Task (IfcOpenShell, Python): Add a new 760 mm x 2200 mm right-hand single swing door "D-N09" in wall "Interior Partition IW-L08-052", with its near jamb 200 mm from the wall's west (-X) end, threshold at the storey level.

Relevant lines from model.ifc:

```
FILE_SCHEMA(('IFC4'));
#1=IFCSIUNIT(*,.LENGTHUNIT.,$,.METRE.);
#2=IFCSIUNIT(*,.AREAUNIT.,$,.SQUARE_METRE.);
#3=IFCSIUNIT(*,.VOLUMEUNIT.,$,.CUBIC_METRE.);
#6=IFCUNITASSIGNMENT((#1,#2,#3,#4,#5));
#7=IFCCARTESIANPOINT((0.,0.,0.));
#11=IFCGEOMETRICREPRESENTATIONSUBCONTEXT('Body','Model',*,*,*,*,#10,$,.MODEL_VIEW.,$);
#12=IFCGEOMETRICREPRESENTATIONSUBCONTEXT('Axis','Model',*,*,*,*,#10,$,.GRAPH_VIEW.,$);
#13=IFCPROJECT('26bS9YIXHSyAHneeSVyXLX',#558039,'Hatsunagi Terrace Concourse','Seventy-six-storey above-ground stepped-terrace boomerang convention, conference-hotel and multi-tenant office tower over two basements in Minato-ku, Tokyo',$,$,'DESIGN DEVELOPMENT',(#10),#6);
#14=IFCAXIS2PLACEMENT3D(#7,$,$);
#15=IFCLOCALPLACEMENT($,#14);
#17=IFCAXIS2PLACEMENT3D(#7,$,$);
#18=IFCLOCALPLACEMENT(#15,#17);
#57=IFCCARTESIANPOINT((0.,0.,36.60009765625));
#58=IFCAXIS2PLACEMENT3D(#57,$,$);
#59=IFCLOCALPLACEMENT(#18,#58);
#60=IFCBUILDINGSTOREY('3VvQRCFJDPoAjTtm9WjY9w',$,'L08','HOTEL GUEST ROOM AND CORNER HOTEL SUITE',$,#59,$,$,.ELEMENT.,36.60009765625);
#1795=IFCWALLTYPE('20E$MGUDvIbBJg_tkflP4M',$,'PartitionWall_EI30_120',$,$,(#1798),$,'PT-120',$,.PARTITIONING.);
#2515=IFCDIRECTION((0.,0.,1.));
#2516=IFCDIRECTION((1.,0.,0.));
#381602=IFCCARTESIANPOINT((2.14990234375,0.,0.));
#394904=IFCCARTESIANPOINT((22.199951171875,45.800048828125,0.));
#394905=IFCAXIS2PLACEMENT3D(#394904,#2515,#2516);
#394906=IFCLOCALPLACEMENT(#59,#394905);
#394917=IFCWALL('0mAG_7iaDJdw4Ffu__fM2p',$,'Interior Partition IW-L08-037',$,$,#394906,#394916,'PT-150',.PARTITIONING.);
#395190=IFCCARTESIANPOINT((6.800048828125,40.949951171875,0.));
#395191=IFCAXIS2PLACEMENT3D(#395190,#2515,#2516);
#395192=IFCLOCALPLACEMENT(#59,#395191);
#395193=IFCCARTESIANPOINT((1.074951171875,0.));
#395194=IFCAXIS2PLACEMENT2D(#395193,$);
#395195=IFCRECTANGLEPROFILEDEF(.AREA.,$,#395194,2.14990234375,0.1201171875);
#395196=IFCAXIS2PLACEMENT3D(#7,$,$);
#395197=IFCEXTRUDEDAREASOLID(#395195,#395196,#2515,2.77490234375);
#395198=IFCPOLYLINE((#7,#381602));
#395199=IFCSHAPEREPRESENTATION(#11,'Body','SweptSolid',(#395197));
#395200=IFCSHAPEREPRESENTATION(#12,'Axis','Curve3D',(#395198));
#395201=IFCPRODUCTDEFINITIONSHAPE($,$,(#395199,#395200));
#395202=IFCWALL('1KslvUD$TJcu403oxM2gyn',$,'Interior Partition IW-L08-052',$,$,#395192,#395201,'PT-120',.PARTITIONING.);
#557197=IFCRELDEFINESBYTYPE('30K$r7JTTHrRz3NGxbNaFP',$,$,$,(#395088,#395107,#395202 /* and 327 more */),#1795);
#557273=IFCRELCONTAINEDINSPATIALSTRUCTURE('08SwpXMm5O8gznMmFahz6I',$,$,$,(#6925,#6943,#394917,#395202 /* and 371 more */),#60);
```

```python
import numpy as np
import ifcopenshell
import ifcopenshell.api.feature
import ifcopenshell.api.geometry
import ifcopenshell.api.root
import ifcopenshell.api.spatial
import ifcopenshell.geom
import ifcopenshell.util.element
import ifcopenshell.util.placement
import ifcopenshell.util.representation
import ifcopenshell.util.shape
import ifcopenshell.util.unit

model = ifcopenshell.open("model.ifc")
unit_scale = ifcopenshell.util.unit.calculate_unit_scale(model)
settings = ifcopenshell.geom.settings()


def volume(element):
    """Net volume in cubic metres, openings subtracted."""
    shape = ifcopenshell.geom.create_shape(settings, element)
    return ifcopenshell.util.shape.get_volume(shape.geometry)


wall = model.by_guid("1KslvUD$TJcu403oxM2gyn")
storey = ifcopenshell.util.element.get_container(wall, ifc_class="IfcBuildingStorey")
context = ifcopenshell.util.representation.get_context(model, "Model", "Body", "MODEL_VIEW")
before = volume(wall)

width, height, from_end, sill = 0.76, 2.2, 0.2, 0.0  # metres

# The wall runs along its own X axis, and the end named is its -X end.
wall_shape = ifcopenshell.geom.create_shape(settings, wall)
x, y, z = ifcopenshell.util.shape.get_vertices(wall_shape.geometry).T
start = x.min() + from_end
face, thickness = float(y.min()), float(y.max() - y.min())
wall_matrix = ifcopenshell.util.placement.get_local_placement(wall.ObjectPlacement)
level = ifcopenshell.util.placement.get_local_placement(storey.ObjectPlacement)[2, 3]


def in_wall(x, y):
    """Placement at x, y metres in the wall's axes, at sill height."""
    matrix = wall_matrix.copy()
    matrix[:, 3] = wall_matrix @ np.array([x / unit_scale, y / unit_scale, 0.0, 1.0])
    matrix[2, 3] = level + sill / unit_scale
    return matrix


# Opening: a box that overshoots both wall faces by 50 mm.
opening = ifcopenshell.api.root.create_entity(model, ifc_class="IfcOpeningElement", predefined_type="OPENING")
box = ifcopenshell.api.geometry.add_wall_representation(
    model, context=context, length=width, height=height, thickness=thickness + 0.1
)
ifcopenshell.api.geometry.assign_representation(model, product=opening, representation=box)
ifcopenshell.api.geometry.edit_object_placement(model, product=opening, matrix=in_wall(start, face - 0.05), is_si=False)
ifcopenshell.api.feature.add_feature(model, feature=opening, element=wall)

door = ifcopenshell.api.root.create_entity(model, ifc_class="IfcDoor", name="D-N09", predefined_type="DOOR")
door.OverallWidth, door.OverallHeight = width / unit_scale, height / unit_scale
door.OperationType = "SINGLE_SWING_RIGHT"
body = ifcopenshell.api.geometry.add_door_representation(
    model,
    context=context,
    overall_width=door.OverallWidth,
    overall_height=door.OverallHeight,
    operation_type="SINGLE_SWING_RIGHT",
    lining_properties={"LiningDepth": thickness / unit_scale, "ThresholdDepth": thickness / unit_scale},
)
ifcopenshell.api.geometry.assign_representation(model, product=door, representation=body)
ifcopenshell.api.spatial.assign_container(model, products=[door], relating_structure=storey)
ifcopenshell.api.feature.add_filling(model, opening=opening, element=door)

# The lining spans the wall, so the door starts at the wall face.
ifcopenshell.api.geometry.edit_object_placement(model, product=door, matrix=in_wall(start, face), is_si=False)

after = volume(wall)

print(f"wall volume {before:.3f} -> {after:.3f} m3")

model.write("model_edited.ifc")
```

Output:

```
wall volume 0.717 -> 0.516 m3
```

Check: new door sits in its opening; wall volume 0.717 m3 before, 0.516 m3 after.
